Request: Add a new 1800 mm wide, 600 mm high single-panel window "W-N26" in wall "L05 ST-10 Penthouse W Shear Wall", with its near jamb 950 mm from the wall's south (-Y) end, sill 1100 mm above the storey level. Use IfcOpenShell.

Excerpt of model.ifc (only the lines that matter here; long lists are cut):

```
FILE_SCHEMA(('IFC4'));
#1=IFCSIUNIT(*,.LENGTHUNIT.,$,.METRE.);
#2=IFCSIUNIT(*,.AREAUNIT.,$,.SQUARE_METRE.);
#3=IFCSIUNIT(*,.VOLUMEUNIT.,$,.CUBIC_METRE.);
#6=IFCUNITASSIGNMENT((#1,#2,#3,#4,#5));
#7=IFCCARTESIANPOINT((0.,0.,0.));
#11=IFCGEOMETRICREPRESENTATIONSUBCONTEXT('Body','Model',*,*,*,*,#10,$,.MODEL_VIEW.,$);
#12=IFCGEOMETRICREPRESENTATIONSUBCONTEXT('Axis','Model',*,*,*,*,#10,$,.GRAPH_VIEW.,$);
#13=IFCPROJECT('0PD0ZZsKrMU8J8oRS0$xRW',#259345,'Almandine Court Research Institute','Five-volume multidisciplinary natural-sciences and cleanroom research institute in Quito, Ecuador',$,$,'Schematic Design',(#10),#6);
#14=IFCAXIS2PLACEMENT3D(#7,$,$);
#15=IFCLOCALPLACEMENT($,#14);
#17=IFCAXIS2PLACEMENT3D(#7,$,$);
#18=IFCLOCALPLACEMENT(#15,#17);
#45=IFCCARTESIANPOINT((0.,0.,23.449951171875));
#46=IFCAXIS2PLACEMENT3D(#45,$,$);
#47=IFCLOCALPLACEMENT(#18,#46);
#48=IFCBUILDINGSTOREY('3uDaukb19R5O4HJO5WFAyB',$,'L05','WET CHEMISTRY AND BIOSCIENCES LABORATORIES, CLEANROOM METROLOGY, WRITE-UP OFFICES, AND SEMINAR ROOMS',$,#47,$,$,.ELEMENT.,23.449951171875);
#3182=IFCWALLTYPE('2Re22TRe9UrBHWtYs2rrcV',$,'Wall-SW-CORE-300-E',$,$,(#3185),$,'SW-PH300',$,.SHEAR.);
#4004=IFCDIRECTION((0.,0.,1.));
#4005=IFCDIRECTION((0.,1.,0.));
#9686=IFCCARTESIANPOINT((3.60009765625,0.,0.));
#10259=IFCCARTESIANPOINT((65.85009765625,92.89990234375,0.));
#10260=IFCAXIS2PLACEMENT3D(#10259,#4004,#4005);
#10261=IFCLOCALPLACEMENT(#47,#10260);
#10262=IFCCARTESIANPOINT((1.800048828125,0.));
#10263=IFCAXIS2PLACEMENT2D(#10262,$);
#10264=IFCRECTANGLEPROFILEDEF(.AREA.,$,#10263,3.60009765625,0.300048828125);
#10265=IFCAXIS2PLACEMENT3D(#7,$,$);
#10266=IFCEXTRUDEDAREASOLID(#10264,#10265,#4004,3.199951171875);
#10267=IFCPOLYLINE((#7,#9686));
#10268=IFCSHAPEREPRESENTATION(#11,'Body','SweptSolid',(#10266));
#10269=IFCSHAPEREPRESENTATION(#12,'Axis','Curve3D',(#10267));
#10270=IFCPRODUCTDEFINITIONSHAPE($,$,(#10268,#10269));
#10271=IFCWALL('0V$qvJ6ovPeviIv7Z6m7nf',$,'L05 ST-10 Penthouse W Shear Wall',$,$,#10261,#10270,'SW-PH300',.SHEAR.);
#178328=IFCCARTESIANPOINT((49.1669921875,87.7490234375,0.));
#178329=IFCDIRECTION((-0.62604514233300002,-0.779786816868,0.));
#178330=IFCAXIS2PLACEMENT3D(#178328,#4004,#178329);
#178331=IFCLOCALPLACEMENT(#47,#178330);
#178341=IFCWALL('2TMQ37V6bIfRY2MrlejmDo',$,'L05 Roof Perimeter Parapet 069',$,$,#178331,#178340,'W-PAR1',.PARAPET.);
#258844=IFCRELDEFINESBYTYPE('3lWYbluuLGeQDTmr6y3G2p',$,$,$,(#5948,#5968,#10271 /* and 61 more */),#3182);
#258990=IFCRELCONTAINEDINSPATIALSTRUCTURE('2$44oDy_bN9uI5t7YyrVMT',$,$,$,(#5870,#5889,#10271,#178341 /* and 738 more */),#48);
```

```python
import numpy as np
import ifcopenshell
import ifcopenshell.api.feature
import ifcopenshell.api.geometry
import ifcopenshell.api.root
import ifcopenshell.api.spatial
import ifcopenshell.geom
import ifcopenshell.util.element
import ifcopenshell.util.placement
import ifcopenshell.util.representation
import ifcopenshell.util.shape
import ifcopenshell.util.unit

model = ifcopenshell.open("model.ifc")
unit_scale = ifcopenshell.util.unit.calculate_unit_scale(model)
settings = ifcopenshell.geom.settings()


def volume(element):
    """Net volume in cubic metres, openings subtracted."""
    shape = ifcopenshell.geom.create_shape(settings, element)
    return ifcopenshell.util.shape.get_volume(shape.geometry)


wall = model.by_guid("0V$qvJ6ovPeviIv7Z6m7nf")
storey = ifcopenshell.util.element.get_container(wall, ifc_class="IfcBuildingStorey")
context = ifcopenshell.util.representation.get_context(model, "Model", "Body", "MODEL_VIEW")
before = volume(wall)

width, height, from_end, sill = 1.8, 0.6, 0.95, 1.1  # metres

# The wall runs along its own X axis, and the end named is its -X end.
wall_shape = ifcopenshell.geom.create_shape(settings, wall)
x, y, z = ifcopenshell.util.shape.get_vertices(wall_shape.geometry).T
start = x.min() + from_end
face, thickness = float(y.min()), float(y.max() - y.min())
wall_matrix = ifcopenshell.util.placement.get_local_placement(wall.ObjectPlacement)
level = ifcopenshell.util.placement.get_local_placement(storey.ObjectPlacement)[2, 3]


def in_wall(x, y):
    """Placement at x, y metres in the wall's axes, at sill height."""
    matrix = wall_matrix.copy()
    matrix[:, 3] = wall_matrix @ np.array([x / unit_scale, y / unit_scale, 0.0, 1.0])
    matrix[2, 3] = level + sill / unit_scale
    return matrix


# Opening: a box that overshoots both wall faces by 50 mm.
opening = ifcopenshell.api.root.create_entity(model, ifc_class="IfcOpeningElement", predefined_type="OPENING")
box = ifcopenshell.api.geometry.add_wall_representation(
    model, context=context, length=width, height=height, thickness=thickness + 0.1
)
ifcopenshell.api.geometry.assign_representation(model, product=opening, representation=box)
ifcopenshell.api.geometry.edit_object_placement(model, product=opening, matrix=in_wall(start, face - 0.05), is_si=False)
ifcopenshell.api.feature.add_feature(model, feature=opening, element=wall)

window = ifcopenshell.api.root.create_entity(model, ifc_class="IfcWindow", name="W-N26", predefined_type="WINDOW")
window.OverallWidth, window.OverallHeight = width / unit_scale, height / unit_scale
window.PartitioningType = "SINGLE_PANEL"
body = ifcopenshell.api.geometry.add_window_representation(
    model,
    context=context,
    overall_width=window.OverallWidth,
    overall_height=window.OverallHeight,
    partition_type="SINGLE_PANEL",
)
ifcopenshell.api.geometry.assign_representation(model, product=window, representation=body)
ifcopenshell.api.spatial.assign_container(model, products=[window], relating_structure=storey)
ifcopenshell.api.feature.add_filling(model, opening=opening, element=window)

# Centre the window in the wall's thickness.
ifcopenshell.api.geometry.edit_object_placement(model, product=window, matrix=in_wall(start, face), is_si=False)
window_shape = ifcopenshell.geom.create_shape(settings, window)
depth = ifcopenshell.util.shape.get_vertices(window_shape.geometry)[:, 1]
offset = face + thickness / 2 - (depth.min() + depth.max()) / 2
ifcopenshell.api.geometry.edit_object_placement(model, product=window, matrix=in_wall(start, offset), is_si=False)

after = volume(wall)

print(f"wall volume {before:.3f} -> {after:.3f} m3")

model.write("model_rev.ifc")
```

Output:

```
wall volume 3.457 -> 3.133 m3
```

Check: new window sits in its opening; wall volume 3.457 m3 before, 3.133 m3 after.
